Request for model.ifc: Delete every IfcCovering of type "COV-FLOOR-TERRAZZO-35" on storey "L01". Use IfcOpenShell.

First a look at what the model holds.

```python
import ifcopenshell
import ifcopenshell.util.element

model = ifcopenshell.open("model.ifc")
print(model.schema)
storey = next(s for s in model.by_type("IfcBuildingStorey") if s.Name == "L01")
coverings = [e for e in ifcopenshell.util.element.get_decomposition(storey) if e.is_a("IfcCovering")]
seen = {}
for e in coverings:
    element_type = ifcopenshell.util.element.get_type(e)
    name = element_type.Name if element_type not in (None, e) else None
    seen[name] = seen.get(name, 0) + 1
for name, count in sorted(seen.items(), key=str):
    print(count, "x", name)
```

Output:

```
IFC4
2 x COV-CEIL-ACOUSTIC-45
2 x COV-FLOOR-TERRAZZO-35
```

```python
import ifcopenshell
import ifcopenshell.api.root
import ifcopenshell.util.element

model = ifcopenshell.open("model.ifc")

storey = next(s for s in model.by_type("IfcBuildingStorey") if s.Name == "L01")
coverings = [e for e in ifcopenshell.util.element.get_decomposition(storey) if e.is_a("IfcCovering")]
targets = [e for e in coverings if (t := ifcopenshell.util.element.get_type(e)) not in (None, e) and t.Name == "COV-FLOOR-TERRAZZO-35"]

for e in targets:
    ifcopenshell.api.root.remove_product(model, product=e)
print(len(targets), "removed")

model.write("model-out.ifc")
```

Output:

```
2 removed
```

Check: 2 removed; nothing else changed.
